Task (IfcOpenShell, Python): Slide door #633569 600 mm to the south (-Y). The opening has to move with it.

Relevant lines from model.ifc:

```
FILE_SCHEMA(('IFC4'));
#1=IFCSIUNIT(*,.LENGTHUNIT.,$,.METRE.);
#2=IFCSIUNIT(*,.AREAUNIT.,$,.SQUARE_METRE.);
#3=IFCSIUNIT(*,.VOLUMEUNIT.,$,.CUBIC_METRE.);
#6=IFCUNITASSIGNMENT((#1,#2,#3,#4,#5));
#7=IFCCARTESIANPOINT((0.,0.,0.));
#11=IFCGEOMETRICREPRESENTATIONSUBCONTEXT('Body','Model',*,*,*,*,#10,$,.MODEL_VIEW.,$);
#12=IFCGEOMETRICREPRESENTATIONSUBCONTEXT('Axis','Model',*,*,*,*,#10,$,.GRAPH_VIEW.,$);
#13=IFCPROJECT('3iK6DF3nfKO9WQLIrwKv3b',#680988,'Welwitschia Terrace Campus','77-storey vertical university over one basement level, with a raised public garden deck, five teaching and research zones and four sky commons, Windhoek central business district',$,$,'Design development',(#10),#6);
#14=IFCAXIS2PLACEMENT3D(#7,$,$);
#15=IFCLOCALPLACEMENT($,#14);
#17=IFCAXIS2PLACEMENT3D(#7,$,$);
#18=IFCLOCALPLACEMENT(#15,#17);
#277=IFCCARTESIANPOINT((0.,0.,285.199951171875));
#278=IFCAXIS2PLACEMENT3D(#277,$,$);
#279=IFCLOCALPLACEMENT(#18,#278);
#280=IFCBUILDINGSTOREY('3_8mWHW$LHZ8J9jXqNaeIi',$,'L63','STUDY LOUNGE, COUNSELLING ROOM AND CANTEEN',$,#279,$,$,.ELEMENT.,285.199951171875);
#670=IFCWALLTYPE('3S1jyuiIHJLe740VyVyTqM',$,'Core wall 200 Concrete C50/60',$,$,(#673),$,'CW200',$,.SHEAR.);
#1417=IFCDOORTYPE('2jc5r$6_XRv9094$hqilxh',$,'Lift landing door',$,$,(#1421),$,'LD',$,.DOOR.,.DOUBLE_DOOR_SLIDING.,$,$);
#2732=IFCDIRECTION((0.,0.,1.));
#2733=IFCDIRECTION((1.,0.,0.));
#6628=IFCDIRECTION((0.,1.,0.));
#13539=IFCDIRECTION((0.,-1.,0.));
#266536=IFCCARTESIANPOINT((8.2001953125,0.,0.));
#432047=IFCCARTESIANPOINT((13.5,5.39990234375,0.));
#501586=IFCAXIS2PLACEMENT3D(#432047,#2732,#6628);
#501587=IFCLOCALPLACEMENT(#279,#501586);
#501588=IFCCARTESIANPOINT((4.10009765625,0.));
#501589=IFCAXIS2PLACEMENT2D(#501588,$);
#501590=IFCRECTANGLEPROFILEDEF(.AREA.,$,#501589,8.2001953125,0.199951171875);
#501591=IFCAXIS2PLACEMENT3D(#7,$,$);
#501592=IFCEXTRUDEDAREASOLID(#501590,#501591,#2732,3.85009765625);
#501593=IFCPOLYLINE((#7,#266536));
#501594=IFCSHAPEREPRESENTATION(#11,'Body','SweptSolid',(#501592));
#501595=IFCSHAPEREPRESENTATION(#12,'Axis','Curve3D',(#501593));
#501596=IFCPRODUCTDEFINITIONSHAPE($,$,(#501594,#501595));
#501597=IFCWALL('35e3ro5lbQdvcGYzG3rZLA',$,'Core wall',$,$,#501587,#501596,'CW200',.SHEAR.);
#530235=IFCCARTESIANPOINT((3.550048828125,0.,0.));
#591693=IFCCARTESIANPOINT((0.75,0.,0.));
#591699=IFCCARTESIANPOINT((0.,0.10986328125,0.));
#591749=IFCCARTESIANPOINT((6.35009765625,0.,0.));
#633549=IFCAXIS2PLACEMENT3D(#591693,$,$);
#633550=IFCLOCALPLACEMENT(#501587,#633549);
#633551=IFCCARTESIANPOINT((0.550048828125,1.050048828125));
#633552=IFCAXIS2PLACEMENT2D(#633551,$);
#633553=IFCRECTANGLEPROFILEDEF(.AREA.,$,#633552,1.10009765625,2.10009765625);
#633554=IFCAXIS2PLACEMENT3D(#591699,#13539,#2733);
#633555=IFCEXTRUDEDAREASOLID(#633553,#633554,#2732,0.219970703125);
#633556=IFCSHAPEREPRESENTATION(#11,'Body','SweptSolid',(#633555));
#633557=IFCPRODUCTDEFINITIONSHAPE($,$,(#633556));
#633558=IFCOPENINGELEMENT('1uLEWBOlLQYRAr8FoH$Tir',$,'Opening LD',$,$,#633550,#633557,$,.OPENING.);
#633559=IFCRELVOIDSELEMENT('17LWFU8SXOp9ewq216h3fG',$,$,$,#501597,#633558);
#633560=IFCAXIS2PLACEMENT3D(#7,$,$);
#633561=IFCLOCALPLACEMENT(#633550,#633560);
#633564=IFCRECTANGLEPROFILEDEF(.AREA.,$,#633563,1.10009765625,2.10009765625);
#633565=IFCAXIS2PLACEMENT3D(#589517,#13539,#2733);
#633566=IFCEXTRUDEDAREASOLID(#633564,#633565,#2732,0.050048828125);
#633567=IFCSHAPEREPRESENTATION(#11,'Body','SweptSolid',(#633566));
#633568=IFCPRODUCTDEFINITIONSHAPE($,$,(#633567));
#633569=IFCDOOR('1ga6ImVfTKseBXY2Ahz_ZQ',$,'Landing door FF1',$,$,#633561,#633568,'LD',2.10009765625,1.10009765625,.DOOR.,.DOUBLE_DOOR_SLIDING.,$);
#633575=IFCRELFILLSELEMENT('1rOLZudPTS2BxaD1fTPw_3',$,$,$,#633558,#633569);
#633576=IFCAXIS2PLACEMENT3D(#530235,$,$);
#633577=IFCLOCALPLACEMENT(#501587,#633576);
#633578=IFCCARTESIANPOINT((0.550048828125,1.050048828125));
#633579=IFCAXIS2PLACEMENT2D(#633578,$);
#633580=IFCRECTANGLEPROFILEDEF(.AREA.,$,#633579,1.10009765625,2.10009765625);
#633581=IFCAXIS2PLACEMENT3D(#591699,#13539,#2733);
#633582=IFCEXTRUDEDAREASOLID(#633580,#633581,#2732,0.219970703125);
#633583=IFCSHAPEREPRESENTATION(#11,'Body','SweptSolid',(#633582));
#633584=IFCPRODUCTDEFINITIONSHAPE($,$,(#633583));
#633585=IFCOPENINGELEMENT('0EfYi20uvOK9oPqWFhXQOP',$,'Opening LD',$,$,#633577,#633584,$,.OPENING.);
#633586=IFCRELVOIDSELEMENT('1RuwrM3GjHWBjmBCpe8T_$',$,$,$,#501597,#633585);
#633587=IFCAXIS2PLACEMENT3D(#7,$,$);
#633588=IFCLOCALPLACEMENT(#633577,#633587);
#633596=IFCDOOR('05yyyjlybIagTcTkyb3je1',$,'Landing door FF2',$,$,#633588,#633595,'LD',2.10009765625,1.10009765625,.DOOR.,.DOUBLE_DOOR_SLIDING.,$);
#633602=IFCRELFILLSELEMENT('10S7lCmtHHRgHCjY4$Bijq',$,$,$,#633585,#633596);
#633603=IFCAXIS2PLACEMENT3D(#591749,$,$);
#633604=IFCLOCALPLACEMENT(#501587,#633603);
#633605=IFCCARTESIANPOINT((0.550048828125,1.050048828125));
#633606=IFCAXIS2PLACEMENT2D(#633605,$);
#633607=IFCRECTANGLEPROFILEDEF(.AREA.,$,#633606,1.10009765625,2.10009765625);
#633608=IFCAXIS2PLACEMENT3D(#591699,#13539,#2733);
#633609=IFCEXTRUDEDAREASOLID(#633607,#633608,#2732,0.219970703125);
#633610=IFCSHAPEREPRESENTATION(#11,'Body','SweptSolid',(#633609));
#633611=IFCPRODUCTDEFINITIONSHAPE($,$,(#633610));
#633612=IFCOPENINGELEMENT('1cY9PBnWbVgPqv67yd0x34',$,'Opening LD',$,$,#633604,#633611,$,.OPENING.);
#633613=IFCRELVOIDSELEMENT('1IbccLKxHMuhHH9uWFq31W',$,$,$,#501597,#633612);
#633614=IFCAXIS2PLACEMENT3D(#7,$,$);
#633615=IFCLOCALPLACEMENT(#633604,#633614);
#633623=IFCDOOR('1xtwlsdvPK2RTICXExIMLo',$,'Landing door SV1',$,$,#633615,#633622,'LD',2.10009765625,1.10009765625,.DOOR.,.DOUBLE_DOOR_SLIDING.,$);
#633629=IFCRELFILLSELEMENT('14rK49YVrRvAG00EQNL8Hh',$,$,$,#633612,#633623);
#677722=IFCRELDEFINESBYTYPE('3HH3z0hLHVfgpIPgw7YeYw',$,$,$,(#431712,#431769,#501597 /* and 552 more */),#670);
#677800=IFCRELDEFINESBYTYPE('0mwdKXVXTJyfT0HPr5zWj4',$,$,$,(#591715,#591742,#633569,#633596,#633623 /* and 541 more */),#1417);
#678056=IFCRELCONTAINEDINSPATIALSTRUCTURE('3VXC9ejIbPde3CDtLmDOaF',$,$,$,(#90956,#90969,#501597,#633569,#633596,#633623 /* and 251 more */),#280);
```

```python
import ifcopenshell
import ifcopenshell.api.geometry
import ifcopenshell.util.placement
import ifcopenshell.util.unit

model = ifcopenshell.open("model.ifc")
unit_scale = ifcopenshell.util.unit.calculate_unit_scale(model)

door = model.by_guid("1ga6ImVfTKseBXY2Ahz_ZQ")
opening = door.FillsVoids[0].RelatingOpeningElement
wall = opening.VoidsElements[0].RelatingBuildingElement

wall_matrix = ifcopenshell.util.placement.get_local_placement(wall.ObjectPlacement)
shift = wall_matrix[:3, 0] * -0.6 / unit_scale
before = ifcopenshell.util.placement.get_local_placement(door.ObjectPlacement)[:3, 3].copy()

# The door is placed relative to its opening, so it follows when the opening moves.
matrix = ifcopenshell.util.placement.get_local_placement(opening.ObjectPlacement)
matrix[:3, 3] += shift
ifcopenshell.api.geometry.edit_object_placement(
    model, product=opening, matrix=matrix, is_si=False, should_transform_children=True
)

after = ifcopenshell.util.placement.get_local_placement(door.ObjectPlacement)[:3, 3]
print("door moved by", (after - before).round(3) + 0.0)

model.write("model_updated.ifc")
```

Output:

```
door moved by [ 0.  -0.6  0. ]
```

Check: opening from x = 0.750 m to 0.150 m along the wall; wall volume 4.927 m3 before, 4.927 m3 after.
